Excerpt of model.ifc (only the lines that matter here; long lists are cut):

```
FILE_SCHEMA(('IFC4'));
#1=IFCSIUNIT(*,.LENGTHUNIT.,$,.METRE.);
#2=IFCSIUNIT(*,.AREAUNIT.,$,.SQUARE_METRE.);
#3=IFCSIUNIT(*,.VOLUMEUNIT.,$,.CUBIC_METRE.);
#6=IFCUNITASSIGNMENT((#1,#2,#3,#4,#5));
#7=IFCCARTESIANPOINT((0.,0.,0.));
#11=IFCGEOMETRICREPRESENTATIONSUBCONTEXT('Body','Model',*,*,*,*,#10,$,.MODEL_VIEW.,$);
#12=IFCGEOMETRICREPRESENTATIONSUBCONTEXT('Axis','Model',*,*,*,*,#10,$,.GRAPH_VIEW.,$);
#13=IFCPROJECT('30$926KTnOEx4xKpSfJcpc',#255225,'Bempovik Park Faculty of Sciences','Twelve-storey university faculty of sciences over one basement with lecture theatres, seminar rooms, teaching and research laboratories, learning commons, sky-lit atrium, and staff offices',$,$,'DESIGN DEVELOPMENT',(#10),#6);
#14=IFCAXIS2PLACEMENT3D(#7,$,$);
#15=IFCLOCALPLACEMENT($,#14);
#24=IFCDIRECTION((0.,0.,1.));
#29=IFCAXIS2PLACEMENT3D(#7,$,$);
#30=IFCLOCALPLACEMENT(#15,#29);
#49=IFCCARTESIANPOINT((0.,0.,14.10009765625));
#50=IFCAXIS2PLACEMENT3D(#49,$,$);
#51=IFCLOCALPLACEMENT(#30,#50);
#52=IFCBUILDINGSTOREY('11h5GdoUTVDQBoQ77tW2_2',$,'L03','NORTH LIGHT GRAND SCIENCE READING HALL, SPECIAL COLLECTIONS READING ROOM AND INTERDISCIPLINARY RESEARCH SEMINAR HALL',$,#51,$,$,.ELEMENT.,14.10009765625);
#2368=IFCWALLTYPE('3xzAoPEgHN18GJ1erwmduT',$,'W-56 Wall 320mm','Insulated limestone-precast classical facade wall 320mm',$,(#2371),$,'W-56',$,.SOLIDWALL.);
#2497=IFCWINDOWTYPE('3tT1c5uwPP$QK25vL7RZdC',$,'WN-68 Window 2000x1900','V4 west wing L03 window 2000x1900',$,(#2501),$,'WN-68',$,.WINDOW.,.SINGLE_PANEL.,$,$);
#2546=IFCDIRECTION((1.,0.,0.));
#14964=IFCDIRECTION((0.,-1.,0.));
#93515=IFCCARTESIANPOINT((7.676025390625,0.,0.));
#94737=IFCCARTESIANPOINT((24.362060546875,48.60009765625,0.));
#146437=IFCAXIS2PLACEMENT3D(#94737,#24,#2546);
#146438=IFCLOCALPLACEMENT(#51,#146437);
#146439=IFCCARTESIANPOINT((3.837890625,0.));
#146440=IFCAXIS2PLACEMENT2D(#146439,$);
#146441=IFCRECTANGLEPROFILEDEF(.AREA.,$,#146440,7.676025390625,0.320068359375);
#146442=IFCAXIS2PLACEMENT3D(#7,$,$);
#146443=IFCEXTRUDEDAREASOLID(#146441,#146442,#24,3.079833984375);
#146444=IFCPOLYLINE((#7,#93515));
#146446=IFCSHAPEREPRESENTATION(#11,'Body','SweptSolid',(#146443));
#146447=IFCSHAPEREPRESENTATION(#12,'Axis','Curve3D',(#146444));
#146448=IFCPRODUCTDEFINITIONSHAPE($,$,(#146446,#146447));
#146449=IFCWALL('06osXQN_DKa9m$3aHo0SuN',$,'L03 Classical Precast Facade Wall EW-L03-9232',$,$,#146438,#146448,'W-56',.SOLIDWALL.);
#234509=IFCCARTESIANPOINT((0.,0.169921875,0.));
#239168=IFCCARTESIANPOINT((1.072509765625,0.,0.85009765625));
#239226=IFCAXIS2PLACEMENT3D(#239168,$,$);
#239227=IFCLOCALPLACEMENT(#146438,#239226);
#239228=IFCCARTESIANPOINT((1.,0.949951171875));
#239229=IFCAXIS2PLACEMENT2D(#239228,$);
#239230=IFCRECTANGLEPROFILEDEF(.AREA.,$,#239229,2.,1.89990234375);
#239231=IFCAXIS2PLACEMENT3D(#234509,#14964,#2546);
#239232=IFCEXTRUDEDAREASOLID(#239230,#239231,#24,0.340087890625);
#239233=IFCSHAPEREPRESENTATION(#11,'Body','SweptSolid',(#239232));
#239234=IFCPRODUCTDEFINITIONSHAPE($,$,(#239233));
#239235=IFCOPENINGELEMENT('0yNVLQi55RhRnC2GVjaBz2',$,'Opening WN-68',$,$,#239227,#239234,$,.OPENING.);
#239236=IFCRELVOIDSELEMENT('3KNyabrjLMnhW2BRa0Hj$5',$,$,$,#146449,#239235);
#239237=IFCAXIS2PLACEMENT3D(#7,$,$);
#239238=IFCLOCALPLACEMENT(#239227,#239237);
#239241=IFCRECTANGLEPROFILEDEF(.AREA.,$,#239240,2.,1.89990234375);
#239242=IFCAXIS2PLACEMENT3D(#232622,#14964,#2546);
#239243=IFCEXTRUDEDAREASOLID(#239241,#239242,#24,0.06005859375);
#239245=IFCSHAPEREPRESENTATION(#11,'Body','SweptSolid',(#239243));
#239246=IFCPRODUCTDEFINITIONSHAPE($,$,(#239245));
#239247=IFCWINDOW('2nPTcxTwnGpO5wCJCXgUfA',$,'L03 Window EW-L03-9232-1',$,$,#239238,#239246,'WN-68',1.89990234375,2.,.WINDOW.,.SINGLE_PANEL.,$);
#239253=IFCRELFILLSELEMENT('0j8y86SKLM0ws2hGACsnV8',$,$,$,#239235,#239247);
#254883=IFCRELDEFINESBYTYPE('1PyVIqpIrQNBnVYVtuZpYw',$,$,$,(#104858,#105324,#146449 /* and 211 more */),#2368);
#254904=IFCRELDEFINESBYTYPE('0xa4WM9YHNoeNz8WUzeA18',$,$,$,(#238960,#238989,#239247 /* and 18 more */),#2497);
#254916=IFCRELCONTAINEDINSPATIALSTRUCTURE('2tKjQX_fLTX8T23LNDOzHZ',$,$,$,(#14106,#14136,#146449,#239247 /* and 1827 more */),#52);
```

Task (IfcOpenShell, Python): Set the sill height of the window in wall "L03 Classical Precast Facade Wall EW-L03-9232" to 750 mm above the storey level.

```python
import numpy as np
import ifcopenshell
import ifcopenshell.api.geometry
import ifcopenshell.geom
import ifcopenshell.util.element
import ifcopenshell.util.placement
import ifcopenshell.util.shape
import ifcopenshell.util.unit

model = ifcopenshell.open("model.ifc")
unit_scale = ifcopenshell.util.unit.calculate_unit_scale(model)

window = model.by_guid("2nPTcxTwnGpO5wCJCXgUfA")
opening = window.FillsVoids[0].RelatingOpeningElement
storey = ifcopenshell.util.element.get_container(window, ifc_class="IfcBuildingStorey")
level = ifcopenshell.util.placement.get_local_placement(storey.ObjectPlacement)[2, 3]

# The opening's origin need not be at the sill, so measure its lowest point.
shape = ifcopenshell.geom.create_shape(ifcopenshell.geom.settings(), opening)
bottom = ifcopenshell.util.shape.get_shape_bottom_elevation(shape, shape.geometry) / unit_scale
dz = level + 0.75 - bottom

shift = np.array([0.0, 0.0, dz])
# The window is placed relative to its opening, so it follows when the opening moves.
matrix = ifcopenshell.util.placement.get_local_placement(opening.ObjectPlacement)
matrix[:3, 3] += shift
ifcopenshell.api.geometry.edit_object_placement(
    model, product=opening, matrix=matrix, is_si=False, should_transform_children=True
)

print(f"moved by {dz * unit_scale:+.3f} m")

model.write("model_edited.ifc")
```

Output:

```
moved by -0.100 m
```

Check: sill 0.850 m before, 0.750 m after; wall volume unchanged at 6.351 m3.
